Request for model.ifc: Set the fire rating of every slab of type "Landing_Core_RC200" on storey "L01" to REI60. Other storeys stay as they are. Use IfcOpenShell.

First a look at what the model holds.

```python
import ifcopenshell
import ifcopenshell.util.element

model = ifcopenshell.open("model.ifc")
print(model.schema)
storey = next(s for s in model.by_type("IfcBuildingStorey") if s.Name == "L01")
slabs = [e for e in ifcopenshell.util.element.get_decomposition(storey) if e.is_a("IfcSlab")]
seen = {}
for e in slabs:
    element_type = ifcopenshell.util.element.get_type(e)
    key = (element_type.Name if element_type != e and element_type else None, ifcopenshell.util.element.get_pset(e, "Pset_SlabCommon", "FireRating"))
    seen[key] = seen.get(key, 0) + 1
for (name, value), count in sorted(seen.items(), key=str):
    print(count, "x", name, "|", value)
```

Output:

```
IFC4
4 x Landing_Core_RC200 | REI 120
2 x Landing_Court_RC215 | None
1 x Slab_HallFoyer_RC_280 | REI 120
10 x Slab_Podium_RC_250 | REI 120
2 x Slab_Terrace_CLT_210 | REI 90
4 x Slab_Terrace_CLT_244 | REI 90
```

```python
import ifcopenshell
import ifcopenshell.api.pset
import ifcopenshell.util.element

model = ifcopenshell.open("model.ifc")

storey = next(s for s in model.by_type("IfcBuildingStorey") if s.Name == "L01")
slabs = [e for e in ifcopenshell.util.element.get_decomposition(storey) if e.is_a("IfcSlab")]

count = 0
for e in slabs:
    element_type = ifcopenshell.util.element.get_type(e)
    if element_type in (None, e) or element_type.Name != "Landing_Core_RC200":
        continue
    # add_pset returns the element's existing set when there is one.
    pset = ifcopenshell.api.pset.add_pset(model, product=e, name="Pset_SlabCommon")
    ifcopenshell.api.pset.edit_pset(model, pset=pset, properties={"FireRating": "REI60"})
    count += 1

print(count, "slabs updated")

model.write("model_v2.ifc")
```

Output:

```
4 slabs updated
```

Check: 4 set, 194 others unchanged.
